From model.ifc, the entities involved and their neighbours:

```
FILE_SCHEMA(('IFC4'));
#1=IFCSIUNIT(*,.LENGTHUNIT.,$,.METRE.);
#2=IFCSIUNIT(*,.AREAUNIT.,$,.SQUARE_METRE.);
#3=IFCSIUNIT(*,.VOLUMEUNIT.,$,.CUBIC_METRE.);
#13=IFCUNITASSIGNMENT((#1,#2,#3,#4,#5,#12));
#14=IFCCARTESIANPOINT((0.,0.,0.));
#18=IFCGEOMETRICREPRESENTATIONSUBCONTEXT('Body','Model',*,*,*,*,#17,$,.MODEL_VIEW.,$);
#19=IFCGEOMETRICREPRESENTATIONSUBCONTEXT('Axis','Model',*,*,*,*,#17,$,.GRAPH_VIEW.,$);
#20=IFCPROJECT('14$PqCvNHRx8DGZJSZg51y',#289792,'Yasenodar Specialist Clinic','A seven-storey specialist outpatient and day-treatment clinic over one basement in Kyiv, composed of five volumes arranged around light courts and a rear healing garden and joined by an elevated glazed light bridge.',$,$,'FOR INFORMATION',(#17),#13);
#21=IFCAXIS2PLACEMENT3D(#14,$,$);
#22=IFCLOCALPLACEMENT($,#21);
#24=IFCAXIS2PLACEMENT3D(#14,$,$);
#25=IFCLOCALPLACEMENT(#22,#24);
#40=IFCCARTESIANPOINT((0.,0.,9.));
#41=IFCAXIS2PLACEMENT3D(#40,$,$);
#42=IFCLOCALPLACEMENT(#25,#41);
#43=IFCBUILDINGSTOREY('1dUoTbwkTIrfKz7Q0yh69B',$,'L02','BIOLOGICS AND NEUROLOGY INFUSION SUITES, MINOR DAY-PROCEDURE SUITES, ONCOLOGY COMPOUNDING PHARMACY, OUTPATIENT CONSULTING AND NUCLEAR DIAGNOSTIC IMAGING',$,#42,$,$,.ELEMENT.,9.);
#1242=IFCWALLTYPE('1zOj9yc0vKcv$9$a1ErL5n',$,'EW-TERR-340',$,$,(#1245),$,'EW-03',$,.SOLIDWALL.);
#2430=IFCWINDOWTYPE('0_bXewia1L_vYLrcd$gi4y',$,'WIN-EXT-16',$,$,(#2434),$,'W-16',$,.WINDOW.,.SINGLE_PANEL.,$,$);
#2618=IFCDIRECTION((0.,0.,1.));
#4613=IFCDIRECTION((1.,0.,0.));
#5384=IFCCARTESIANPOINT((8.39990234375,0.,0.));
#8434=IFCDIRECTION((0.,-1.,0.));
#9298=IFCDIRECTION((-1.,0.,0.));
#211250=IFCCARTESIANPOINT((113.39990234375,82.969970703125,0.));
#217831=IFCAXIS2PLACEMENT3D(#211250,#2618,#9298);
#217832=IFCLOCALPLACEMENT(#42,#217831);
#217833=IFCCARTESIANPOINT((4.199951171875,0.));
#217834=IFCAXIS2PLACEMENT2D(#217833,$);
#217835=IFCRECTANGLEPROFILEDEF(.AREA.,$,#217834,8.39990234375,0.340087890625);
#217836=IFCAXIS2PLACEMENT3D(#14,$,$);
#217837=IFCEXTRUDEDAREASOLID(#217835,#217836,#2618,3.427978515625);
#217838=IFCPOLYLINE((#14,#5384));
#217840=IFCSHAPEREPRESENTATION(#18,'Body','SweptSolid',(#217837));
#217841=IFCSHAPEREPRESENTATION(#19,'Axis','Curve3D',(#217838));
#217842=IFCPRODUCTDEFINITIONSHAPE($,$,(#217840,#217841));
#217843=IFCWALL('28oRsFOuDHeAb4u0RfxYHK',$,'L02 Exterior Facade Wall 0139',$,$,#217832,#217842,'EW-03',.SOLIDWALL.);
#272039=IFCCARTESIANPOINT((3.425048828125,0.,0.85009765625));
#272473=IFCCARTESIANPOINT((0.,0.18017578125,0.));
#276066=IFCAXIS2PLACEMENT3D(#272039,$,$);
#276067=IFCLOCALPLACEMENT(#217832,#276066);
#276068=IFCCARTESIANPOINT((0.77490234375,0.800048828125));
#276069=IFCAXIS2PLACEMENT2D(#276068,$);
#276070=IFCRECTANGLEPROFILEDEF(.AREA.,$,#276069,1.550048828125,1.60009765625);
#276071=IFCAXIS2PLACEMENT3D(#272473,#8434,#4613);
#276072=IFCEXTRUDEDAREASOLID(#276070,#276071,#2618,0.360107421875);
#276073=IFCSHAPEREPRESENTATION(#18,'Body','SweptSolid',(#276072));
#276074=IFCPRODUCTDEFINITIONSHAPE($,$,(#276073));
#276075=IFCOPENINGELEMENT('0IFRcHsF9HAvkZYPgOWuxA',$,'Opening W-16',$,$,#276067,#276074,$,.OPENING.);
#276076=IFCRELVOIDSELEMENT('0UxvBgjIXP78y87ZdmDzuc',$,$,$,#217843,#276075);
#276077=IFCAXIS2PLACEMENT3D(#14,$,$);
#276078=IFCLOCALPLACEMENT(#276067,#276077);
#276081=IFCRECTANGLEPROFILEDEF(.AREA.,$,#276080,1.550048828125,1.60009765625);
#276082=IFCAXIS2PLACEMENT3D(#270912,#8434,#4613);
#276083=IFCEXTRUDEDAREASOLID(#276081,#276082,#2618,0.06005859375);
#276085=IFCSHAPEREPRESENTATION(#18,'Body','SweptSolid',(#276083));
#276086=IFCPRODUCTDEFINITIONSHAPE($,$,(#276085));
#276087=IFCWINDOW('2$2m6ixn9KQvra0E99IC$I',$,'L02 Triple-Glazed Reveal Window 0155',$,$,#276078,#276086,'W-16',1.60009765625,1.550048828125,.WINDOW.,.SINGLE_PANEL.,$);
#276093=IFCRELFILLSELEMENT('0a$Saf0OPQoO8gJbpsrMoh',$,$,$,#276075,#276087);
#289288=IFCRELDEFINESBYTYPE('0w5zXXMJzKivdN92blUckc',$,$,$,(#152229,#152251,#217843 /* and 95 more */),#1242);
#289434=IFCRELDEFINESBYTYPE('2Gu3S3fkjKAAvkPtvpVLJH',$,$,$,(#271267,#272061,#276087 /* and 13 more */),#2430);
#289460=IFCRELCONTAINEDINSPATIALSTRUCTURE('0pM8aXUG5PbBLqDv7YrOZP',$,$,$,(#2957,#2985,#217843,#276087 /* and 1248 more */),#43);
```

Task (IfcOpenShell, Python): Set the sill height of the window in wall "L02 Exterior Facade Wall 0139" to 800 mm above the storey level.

```python
import numpy as np
import ifcopenshell
import ifcopenshell.api.geometry
import ifcopenshell.geom
import ifcopenshell.util.element
import ifcopenshell.util.placement
import ifcopenshell.util.shape
import ifcopenshell.util.unit

model = ifcopenshell.open("model.ifc")
unit_scale = ifcopenshell.util.unit.calculate_unit_scale(model)

window = model.by_id(276087)
opening = window.FillsVoids[0].RelatingOpeningElement
storey = ifcopenshell.util.element.get_container(window, ifc_class="IfcBuildingStorey")
level = ifcopenshell.util.placement.get_local_placement(storey.ObjectPlacement)[2, 3]

# The opening's origin need not be at the sill, so measure its lowest point.
shape = ifcopenshell.geom.create_shape(ifcopenshell.geom.settings(), opening)
bottom = ifcopenshell.util.shape.get_shape_bottom_elevation(shape, shape.geometry) / unit_scale
dz = level + 0.8 - bottom

shift = np.array([0.0, 0.0, dz])
# The window is placed relative to its opening, so it follows when the opening moves.
matrix = ifcopenshell.util.placement.get_local_placement(opening.ObjectPlacement)
matrix[:3, 3] += shift
ifcopenshell.api.geometry.edit_object_placement(
    model, product=opening, matrix=matrix, is_si=False, should_transform_children=True
)

print(f"moved by {dz * unit_scale:+.3f} m")

model.write("model_edited.ifc")
```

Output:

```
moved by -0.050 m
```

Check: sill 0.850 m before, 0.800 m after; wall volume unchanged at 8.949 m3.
